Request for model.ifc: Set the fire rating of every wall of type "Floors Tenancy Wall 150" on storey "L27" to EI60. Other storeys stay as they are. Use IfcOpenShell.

First a look at what the model holds.

```python
import ifcopenshell
import ifcopenshell.util.element

model = ifcopenshell.open("model.ifc")
print(model.schema)
storey = next(s for s in model.by_type("IfcBuildingStorey") if s.Name == "L27")
walls = [e for e in ifcopenshell.util.element.get_decomposition(storey) if e.is_a("IfcWall")]
seen = {}
for e in walls:
    element_type = ifcopenshell.util.element.get_type(e)
    key = (element_type.Name if element_type != e and element_type else None, ifcopenshell.util.element.get_pset(e, "Pset_WallCommon", "FireRating"))
    seen[key] = seen.get(key, 0) + 1
for (name, value), count in sorted(seen.items(), key=str):
    print(count, "x", name, "|", value)
```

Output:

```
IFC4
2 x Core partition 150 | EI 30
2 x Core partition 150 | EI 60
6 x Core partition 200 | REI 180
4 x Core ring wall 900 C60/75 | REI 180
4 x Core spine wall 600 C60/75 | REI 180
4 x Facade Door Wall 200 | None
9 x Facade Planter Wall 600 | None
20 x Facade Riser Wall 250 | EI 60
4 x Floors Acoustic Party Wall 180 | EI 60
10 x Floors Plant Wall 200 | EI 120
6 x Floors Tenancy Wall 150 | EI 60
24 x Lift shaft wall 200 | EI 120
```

```python
import ifcopenshell
import ifcopenshell.api.pset
import ifcopenshell.util.element

model = ifcopenshell.open("model.ifc")

storey = next(s for s in model.by_type("IfcBuildingStorey") if s.Name == "L27")
walls = [e for e in ifcopenshell.util.element.get_decomposition(storey) if e.is_a("IfcWall")]

count = 0
for e in walls:
    element_type = ifcopenshell.util.element.get_type(e)
    if element_type in (None, e) or element_type.Name != "Floors Tenancy Wall 150":
        continue
    found = ifcopenshell.util.element.get_pset(e, "Pset_WallCommon", should_inherit=False)
    if found:
        pset = model.by_id(found["id"])
        if len(ifcopenshell.util.element.get_elements_by_pset(pset)) > 1:
            pset = ifcopenshell.api.pset.unshare_pset(model, products=[e], pset=pset)[0]
    else:
        pset = ifcopenshell.api.pset.add_pset(model, product=e, name="Pset_WallCommon")
    ifcopenshell.api.pset.edit_pset(model, pset=pset, properties={"FireRating": "EI60"})
    count += 1

print(count, "walls updated")

model.write("model_v2.ifc")
```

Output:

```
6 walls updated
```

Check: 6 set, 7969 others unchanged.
